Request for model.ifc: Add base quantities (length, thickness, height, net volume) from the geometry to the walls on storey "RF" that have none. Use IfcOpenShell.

First a look at what the model holds.

```python
import ifcopenshell
import ifcopenshell.util.element
import ifcopenshell.util.unit

model = ifcopenshell.open("model.ifc")
print(model.schema)
for unit_type in ("LENGTHUNIT", "AREAUNIT", "VOLUMEUNIT"):
    print(unit_type, ifcopenshell.util.unit.calculate_unit_scale(model, unit_type))
storey = next(s for s in model.by_type("IfcBuildingStorey") if s.Name == "RF")
walls = [e for e in ifcopenshell.util.element.get_decomposition(storey) if e.is_a("IfcWall")]
for e in sorted(walls, key=lambda e: e.id()):
    print(e.id(), e.is_a(), e.Name, list(ifcopenshell.util.element.get_psets(e, qtos_only=True)), sep=" | ")
```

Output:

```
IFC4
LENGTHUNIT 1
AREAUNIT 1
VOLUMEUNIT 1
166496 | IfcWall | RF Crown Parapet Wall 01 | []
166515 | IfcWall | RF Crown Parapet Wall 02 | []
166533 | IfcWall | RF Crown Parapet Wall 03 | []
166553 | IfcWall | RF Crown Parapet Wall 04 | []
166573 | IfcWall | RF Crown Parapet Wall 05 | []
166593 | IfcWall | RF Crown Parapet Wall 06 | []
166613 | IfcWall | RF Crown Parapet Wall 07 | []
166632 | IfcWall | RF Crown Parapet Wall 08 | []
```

```python
import ifcopenshell
import ifcopenshell.api.pset
import ifcopenshell.geom
import ifcopenshell.util.element
import ifcopenshell.util.shape
import ifcopenshell.util.unit

model = ifcopenshell.open("model.ifc")
unit_scale = ifcopenshell.util.unit.calculate_unit_scale(model)
volume_scale = ifcopenshell.util.unit.calculate_unit_scale(model, "VOLUMEUNIT")
settings = ifcopenshell.geom.settings()

storey = next(s for s in model.by_type("IfcBuildingStorey") if s.Name == "RF")
walls = [e for e in ifcopenshell.util.element.get_decomposition(storey) if e.is_a("IfcWall")]

for e in sorted(walls, key=lambda e: e.id()):
    if ifcopenshell.util.element.get_psets(e, qtos_only=True, should_inherit=False):
        continue
    # Geometry comes back in metres, in the element's own axes.
    shape = ifcopenshell.geom.create_shape(settings, e)
    values = {
        "Length": ifcopenshell.util.shape.get_x(shape.geometry) / unit_scale,
        "Width": ifcopenshell.util.shape.get_y(shape.geometry) / unit_scale,
        "Height": ifcopenshell.util.shape.get_z(shape.geometry) / unit_scale,
        "NetVolume": ifcopenshell.util.shape.get_volume(shape.geometry) / volume_scale,
    }
    qto = ifcopenshell.api.pset.add_qto(model, product=e, name="Qto_WallBaseQuantities")
    ifcopenshell.api.pset.edit_qto(model, qto=qto, properties=values)
    print(e.id(), {k: round(v, 3) for k, v in values.items()})

model.write("model_rev.ifc")
```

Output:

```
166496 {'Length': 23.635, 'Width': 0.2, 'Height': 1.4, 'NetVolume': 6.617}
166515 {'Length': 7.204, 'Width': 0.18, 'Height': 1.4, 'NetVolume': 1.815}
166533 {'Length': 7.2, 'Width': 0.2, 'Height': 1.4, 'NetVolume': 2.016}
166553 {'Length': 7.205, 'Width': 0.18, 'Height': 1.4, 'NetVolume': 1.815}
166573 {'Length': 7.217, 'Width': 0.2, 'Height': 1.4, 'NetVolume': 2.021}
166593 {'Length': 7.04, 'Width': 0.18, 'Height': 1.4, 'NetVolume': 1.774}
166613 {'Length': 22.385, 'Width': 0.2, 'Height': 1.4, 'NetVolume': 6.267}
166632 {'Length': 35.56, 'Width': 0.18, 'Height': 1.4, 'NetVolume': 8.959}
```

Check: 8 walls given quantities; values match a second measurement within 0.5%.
